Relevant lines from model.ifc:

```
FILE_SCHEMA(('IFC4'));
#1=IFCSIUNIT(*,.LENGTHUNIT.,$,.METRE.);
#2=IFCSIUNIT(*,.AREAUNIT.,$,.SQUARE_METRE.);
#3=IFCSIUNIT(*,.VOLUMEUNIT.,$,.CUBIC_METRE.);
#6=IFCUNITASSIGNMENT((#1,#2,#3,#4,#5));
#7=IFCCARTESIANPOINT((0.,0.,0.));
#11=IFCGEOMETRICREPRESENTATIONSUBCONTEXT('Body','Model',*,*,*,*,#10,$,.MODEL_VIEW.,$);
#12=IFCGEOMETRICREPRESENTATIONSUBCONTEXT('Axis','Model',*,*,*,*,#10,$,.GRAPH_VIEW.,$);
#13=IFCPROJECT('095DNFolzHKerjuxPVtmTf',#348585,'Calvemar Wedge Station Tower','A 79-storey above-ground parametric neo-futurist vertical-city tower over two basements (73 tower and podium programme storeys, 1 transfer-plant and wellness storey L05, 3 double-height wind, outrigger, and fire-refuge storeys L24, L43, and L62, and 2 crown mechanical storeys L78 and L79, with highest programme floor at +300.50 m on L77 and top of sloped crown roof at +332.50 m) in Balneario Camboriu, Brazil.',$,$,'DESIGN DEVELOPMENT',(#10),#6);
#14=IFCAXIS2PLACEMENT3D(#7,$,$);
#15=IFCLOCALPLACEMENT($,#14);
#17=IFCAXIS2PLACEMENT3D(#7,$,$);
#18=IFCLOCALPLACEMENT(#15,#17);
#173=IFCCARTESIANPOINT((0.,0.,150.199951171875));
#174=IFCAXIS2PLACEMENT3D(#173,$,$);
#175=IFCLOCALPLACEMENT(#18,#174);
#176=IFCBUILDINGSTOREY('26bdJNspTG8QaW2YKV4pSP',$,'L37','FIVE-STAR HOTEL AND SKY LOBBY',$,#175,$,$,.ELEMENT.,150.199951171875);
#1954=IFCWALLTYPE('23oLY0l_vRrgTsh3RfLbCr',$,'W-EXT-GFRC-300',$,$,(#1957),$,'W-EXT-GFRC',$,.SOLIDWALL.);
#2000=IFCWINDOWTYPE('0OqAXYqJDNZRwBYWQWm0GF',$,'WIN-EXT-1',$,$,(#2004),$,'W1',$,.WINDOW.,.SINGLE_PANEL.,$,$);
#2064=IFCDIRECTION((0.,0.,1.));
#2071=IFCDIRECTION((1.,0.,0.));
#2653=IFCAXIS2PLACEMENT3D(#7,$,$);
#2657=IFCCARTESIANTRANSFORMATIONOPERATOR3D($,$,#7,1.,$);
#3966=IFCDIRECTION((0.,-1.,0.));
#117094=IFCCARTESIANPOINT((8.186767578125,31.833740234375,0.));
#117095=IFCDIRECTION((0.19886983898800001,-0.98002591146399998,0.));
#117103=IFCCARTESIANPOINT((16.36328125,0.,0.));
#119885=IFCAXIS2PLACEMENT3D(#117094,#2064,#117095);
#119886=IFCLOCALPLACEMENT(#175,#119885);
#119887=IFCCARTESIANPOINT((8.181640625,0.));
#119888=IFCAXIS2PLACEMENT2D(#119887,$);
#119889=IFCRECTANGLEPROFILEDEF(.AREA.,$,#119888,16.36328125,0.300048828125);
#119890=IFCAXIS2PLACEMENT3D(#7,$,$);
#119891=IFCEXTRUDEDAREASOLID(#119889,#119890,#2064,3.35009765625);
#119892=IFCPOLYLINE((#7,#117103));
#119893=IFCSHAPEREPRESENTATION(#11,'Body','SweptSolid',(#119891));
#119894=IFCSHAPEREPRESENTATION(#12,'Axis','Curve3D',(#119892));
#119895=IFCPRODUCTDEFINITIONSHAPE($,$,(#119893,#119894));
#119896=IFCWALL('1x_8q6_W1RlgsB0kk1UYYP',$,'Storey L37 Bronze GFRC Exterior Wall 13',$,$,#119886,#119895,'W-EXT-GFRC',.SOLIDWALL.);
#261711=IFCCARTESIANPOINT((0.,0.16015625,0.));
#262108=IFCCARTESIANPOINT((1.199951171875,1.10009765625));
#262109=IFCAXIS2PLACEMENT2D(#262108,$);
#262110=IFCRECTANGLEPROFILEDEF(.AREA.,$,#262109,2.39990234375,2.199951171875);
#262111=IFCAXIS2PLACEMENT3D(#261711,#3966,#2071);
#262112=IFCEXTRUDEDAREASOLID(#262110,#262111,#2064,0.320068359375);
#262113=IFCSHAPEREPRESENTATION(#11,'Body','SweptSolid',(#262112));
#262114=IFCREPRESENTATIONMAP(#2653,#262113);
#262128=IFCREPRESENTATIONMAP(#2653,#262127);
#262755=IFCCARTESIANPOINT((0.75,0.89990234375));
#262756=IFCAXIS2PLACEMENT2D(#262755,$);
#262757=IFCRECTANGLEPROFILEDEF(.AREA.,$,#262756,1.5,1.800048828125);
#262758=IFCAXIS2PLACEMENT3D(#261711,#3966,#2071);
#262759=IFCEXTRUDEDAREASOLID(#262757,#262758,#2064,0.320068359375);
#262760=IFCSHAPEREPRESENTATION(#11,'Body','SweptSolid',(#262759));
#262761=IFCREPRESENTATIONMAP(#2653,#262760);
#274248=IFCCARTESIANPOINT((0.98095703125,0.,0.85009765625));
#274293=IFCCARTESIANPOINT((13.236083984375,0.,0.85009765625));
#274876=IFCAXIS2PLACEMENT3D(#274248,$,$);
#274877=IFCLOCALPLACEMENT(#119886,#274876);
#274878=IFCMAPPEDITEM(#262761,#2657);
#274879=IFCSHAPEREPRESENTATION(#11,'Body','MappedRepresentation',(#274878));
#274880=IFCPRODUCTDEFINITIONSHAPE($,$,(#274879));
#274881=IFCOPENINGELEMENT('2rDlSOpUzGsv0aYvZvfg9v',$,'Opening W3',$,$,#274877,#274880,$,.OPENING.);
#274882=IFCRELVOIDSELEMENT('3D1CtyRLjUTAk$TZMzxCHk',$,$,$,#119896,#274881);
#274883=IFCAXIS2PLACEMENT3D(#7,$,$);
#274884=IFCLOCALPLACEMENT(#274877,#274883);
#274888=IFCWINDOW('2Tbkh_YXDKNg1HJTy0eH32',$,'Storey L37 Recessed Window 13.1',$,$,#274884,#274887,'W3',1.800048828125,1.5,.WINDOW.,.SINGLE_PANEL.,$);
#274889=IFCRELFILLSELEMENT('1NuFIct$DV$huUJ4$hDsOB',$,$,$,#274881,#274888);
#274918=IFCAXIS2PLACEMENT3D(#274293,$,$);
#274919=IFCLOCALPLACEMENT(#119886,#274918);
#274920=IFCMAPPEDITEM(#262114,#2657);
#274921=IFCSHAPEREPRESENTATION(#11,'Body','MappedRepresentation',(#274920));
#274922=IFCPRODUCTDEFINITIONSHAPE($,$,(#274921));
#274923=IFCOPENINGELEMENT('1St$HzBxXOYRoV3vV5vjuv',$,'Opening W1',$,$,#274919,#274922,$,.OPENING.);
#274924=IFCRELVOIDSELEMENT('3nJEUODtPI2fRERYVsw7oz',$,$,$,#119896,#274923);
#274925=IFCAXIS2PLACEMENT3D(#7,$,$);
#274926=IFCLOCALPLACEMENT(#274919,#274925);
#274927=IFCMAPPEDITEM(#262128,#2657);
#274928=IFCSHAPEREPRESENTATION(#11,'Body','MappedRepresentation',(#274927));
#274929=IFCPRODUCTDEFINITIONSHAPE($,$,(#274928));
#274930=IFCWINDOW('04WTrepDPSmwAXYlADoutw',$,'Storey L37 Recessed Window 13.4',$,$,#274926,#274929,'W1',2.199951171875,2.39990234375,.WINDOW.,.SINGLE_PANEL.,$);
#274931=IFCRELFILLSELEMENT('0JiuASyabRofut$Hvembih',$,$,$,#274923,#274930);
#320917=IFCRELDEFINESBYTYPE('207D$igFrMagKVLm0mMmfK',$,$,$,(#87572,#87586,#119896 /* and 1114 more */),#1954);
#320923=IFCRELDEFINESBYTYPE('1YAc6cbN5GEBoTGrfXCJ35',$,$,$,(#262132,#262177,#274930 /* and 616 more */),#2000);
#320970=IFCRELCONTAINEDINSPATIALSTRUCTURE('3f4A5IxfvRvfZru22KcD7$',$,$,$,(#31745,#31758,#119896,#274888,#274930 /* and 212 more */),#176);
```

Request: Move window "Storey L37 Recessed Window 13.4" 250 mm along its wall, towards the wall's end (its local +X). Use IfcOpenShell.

```python
import ifcopenshell
import ifcopenshell.api.geometry
import ifcopenshell.util.placement
import ifcopenshell.util.unit

model = ifcopenshell.open("model.ifc")
unit_scale = ifcopenshell.util.unit.calculate_unit_scale(model)

window = model.by_guid("04WTrepDPSmwAXYlADoutw")
opening = window.FillsVoids[0].RelatingOpeningElement
wall = opening.VoidsElements[0].RelatingBuildingElement

wall_matrix = ifcopenshell.util.placement.get_local_placement(wall.ObjectPlacement)
shift = wall_matrix[:3, 0] * 0.25 / unit_scale
before = ifcopenshell.util.placement.get_local_placement(window.ObjectPlacement)[:3, 3].copy()

# The window is placed relative to its opening, so it follows when the opening moves.
matrix = ifcopenshell.util.placement.get_local_placement(opening.ObjectPlacement)
matrix[:3, 3] += shift
ifcopenshell.api.geometry.edit_object_placement(
    model, product=opening, matrix=matrix, is_si=False, should_transform_children=True
)

after = ifcopenshell.util.placement.get_local_placement(window.ObjectPlacement)[:3, 3]
print("window moved by", (after - before).round(3) + 0.0)

model.write("model-out.ifc")
```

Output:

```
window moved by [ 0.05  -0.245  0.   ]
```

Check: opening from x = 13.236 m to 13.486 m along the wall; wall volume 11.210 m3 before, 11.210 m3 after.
